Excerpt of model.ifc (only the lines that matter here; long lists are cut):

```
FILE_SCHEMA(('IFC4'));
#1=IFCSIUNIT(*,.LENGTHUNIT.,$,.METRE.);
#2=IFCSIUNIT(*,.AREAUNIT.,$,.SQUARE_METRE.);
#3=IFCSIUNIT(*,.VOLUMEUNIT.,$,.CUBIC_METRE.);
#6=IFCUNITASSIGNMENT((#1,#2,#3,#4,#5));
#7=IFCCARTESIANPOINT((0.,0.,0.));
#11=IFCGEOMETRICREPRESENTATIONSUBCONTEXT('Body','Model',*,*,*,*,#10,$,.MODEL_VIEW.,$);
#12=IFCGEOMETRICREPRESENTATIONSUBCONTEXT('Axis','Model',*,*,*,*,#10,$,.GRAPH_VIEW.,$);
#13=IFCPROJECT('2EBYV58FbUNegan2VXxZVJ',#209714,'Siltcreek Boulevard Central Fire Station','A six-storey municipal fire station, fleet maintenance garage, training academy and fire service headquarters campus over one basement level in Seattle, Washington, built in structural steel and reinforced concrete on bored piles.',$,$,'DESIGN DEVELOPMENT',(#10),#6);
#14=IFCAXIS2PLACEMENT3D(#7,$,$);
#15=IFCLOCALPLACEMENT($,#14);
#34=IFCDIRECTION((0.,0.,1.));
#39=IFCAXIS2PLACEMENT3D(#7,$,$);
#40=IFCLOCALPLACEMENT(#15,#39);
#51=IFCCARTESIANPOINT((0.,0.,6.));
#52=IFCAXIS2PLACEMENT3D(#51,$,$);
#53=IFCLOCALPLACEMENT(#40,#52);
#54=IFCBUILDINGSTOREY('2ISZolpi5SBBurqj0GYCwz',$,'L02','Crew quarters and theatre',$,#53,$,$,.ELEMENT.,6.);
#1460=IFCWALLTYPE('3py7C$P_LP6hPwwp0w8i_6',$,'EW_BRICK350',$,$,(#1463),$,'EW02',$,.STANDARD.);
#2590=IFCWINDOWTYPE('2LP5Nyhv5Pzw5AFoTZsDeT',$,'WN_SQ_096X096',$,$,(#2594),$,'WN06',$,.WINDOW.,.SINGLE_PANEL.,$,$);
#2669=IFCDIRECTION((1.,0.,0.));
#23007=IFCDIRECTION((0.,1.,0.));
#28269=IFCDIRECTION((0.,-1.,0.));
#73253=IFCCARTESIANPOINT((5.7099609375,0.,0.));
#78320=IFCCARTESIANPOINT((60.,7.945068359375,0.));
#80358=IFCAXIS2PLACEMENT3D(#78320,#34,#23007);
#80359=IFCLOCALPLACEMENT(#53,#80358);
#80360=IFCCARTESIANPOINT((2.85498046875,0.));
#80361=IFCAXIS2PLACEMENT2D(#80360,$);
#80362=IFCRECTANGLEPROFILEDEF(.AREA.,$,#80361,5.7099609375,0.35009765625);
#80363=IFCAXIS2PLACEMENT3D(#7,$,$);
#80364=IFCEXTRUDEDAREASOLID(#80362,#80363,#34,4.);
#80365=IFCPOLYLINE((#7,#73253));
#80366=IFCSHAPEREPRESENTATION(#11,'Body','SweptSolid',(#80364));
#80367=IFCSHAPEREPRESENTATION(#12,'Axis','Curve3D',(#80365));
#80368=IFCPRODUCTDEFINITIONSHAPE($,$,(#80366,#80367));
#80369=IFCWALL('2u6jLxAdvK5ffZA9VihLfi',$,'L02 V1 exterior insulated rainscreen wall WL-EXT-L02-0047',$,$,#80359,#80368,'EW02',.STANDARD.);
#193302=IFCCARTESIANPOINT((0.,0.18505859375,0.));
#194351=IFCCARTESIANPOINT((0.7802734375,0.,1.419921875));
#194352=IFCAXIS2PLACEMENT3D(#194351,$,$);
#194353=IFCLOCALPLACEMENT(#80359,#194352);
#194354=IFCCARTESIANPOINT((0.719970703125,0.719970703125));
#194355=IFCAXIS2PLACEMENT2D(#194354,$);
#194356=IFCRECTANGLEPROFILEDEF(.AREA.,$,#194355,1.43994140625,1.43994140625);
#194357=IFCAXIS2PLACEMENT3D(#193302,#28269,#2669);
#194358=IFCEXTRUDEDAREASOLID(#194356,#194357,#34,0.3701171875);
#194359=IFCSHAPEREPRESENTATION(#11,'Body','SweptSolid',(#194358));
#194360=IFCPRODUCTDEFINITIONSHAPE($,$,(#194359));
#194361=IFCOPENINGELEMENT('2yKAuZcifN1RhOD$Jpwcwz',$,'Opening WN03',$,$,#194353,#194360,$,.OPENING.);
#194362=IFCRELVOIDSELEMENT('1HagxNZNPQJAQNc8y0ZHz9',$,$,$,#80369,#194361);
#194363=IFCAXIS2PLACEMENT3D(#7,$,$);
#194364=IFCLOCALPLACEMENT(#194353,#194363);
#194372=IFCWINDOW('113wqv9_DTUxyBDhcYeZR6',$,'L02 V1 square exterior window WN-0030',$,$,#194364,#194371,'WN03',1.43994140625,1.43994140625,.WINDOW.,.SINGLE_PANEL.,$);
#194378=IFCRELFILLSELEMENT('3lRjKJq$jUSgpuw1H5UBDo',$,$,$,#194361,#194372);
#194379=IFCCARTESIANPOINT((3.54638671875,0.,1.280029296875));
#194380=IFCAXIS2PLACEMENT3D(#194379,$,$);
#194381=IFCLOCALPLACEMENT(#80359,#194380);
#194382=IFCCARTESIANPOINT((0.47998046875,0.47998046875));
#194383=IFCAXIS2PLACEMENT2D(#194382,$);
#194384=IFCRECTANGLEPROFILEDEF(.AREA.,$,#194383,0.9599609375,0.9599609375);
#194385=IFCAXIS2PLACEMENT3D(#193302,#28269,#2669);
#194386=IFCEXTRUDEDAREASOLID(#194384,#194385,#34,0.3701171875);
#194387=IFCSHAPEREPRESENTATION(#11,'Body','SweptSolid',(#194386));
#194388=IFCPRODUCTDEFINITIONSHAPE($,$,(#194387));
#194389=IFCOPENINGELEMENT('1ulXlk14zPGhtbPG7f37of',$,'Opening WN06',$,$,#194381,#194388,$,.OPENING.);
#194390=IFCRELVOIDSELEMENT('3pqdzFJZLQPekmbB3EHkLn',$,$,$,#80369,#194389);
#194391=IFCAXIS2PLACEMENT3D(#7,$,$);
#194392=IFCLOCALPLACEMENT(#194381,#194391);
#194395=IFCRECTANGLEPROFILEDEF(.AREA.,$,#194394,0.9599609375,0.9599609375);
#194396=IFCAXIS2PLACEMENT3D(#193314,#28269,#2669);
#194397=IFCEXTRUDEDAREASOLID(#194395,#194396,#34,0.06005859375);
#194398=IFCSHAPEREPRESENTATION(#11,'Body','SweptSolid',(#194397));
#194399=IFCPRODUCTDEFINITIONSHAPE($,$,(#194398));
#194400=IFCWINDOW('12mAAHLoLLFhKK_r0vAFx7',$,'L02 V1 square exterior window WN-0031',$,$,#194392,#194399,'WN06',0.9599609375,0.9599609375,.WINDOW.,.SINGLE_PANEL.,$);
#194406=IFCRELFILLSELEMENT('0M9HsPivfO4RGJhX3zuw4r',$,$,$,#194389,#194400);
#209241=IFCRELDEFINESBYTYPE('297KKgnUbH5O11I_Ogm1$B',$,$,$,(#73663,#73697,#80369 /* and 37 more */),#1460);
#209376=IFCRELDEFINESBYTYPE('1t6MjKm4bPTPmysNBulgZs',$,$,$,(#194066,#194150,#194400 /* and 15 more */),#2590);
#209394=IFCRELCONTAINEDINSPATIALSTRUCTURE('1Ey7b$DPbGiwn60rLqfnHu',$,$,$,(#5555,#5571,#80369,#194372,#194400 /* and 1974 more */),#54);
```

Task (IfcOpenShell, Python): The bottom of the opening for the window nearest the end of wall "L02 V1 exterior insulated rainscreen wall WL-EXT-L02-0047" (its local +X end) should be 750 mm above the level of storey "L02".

```python
import numpy as np
import ifcopenshell
import ifcopenshell.api.geometry
import ifcopenshell.geom
import ifcopenshell.util.element
import ifcopenshell.util.placement
import ifcopenshell.util.shape
import ifcopenshell.util.unit

model = ifcopenshell.open("model.ifc")
unit_scale = ifcopenshell.util.unit.calculate_unit_scale(model)

window = model.by_guid("12mAAHLoLLFhKK_r0vAFx7")
opening = window.FillsVoids[0].RelatingOpeningElement
storey = ifcopenshell.util.element.get_container(window, ifc_class="IfcBuildingStorey")
level = ifcopenshell.util.placement.get_local_placement(storey.ObjectPlacement)[2, 3]

# The opening's origin need not be at the sill, so measure its lowest point.
shape = ifcopenshell.geom.create_shape(ifcopenshell.geom.settings(), opening)
bottom = ifcopenshell.util.shape.get_shape_bottom_elevation(shape, shape.geometry) / unit_scale
dz = level + 0.75 / unit_scale - bottom

shift = np.array([0.0, 0.0, dz])
# The window is placed relative to its opening, so it follows when the opening moves.
matrix = ifcopenshell.util.placement.get_local_placement(opening.ObjectPlacement)
matrix[:3, 3] += shift
ifcopenshell.api.geometry.edit_object_placement(
    model, product=opening, matrix=matrix, is_si=False, should_transform_children=True
)

print(f"moved by {dz * unit_scale:+.3f} m")

model.write("model_updated.ifc")
```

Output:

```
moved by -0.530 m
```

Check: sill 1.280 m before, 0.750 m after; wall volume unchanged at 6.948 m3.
